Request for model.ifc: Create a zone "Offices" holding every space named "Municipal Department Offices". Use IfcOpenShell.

First a look at what the model holds.

```python
import ifcopenshell

model = ifcopenshell.open("model.ifc")
print(model.schema)
seen = {}
for space in model.by_type("IfcSpace"):
    seen[space.LongName] = seen.get(space.LongName, 0) + 1
for name, count in sorted(seen.items(), key=str):
    print(count, "x", name)
print("zones:", [z.Name for z in model.by_type("IfcZone")][:20])
```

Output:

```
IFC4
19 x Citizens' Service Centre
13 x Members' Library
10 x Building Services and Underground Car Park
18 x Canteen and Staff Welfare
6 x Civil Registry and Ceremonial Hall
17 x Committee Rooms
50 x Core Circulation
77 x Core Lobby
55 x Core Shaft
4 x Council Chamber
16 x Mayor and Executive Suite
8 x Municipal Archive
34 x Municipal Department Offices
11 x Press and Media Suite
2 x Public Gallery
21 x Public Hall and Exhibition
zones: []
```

```python
import ifcopenshell
import ifcopenshell.api.group
import ifcopenshell.api.root

model = ifcopenshell.open("model.ifc")

names = {"Municipal Department Offices"}
spaces = [s for s in model.by_type("IfcSpace") if s.LongName in names]

zone = ifcopenshell.api.root.create_entity(model, ifc_class="IfcZone", name="Offices")
ifcopenshell.api.group.assign_group(model, products=spaces, group=zone)
print(len(spaces), "spaces in", zone.Name)

model.write("model_v2.ifc")
```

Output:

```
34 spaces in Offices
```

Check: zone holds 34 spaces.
